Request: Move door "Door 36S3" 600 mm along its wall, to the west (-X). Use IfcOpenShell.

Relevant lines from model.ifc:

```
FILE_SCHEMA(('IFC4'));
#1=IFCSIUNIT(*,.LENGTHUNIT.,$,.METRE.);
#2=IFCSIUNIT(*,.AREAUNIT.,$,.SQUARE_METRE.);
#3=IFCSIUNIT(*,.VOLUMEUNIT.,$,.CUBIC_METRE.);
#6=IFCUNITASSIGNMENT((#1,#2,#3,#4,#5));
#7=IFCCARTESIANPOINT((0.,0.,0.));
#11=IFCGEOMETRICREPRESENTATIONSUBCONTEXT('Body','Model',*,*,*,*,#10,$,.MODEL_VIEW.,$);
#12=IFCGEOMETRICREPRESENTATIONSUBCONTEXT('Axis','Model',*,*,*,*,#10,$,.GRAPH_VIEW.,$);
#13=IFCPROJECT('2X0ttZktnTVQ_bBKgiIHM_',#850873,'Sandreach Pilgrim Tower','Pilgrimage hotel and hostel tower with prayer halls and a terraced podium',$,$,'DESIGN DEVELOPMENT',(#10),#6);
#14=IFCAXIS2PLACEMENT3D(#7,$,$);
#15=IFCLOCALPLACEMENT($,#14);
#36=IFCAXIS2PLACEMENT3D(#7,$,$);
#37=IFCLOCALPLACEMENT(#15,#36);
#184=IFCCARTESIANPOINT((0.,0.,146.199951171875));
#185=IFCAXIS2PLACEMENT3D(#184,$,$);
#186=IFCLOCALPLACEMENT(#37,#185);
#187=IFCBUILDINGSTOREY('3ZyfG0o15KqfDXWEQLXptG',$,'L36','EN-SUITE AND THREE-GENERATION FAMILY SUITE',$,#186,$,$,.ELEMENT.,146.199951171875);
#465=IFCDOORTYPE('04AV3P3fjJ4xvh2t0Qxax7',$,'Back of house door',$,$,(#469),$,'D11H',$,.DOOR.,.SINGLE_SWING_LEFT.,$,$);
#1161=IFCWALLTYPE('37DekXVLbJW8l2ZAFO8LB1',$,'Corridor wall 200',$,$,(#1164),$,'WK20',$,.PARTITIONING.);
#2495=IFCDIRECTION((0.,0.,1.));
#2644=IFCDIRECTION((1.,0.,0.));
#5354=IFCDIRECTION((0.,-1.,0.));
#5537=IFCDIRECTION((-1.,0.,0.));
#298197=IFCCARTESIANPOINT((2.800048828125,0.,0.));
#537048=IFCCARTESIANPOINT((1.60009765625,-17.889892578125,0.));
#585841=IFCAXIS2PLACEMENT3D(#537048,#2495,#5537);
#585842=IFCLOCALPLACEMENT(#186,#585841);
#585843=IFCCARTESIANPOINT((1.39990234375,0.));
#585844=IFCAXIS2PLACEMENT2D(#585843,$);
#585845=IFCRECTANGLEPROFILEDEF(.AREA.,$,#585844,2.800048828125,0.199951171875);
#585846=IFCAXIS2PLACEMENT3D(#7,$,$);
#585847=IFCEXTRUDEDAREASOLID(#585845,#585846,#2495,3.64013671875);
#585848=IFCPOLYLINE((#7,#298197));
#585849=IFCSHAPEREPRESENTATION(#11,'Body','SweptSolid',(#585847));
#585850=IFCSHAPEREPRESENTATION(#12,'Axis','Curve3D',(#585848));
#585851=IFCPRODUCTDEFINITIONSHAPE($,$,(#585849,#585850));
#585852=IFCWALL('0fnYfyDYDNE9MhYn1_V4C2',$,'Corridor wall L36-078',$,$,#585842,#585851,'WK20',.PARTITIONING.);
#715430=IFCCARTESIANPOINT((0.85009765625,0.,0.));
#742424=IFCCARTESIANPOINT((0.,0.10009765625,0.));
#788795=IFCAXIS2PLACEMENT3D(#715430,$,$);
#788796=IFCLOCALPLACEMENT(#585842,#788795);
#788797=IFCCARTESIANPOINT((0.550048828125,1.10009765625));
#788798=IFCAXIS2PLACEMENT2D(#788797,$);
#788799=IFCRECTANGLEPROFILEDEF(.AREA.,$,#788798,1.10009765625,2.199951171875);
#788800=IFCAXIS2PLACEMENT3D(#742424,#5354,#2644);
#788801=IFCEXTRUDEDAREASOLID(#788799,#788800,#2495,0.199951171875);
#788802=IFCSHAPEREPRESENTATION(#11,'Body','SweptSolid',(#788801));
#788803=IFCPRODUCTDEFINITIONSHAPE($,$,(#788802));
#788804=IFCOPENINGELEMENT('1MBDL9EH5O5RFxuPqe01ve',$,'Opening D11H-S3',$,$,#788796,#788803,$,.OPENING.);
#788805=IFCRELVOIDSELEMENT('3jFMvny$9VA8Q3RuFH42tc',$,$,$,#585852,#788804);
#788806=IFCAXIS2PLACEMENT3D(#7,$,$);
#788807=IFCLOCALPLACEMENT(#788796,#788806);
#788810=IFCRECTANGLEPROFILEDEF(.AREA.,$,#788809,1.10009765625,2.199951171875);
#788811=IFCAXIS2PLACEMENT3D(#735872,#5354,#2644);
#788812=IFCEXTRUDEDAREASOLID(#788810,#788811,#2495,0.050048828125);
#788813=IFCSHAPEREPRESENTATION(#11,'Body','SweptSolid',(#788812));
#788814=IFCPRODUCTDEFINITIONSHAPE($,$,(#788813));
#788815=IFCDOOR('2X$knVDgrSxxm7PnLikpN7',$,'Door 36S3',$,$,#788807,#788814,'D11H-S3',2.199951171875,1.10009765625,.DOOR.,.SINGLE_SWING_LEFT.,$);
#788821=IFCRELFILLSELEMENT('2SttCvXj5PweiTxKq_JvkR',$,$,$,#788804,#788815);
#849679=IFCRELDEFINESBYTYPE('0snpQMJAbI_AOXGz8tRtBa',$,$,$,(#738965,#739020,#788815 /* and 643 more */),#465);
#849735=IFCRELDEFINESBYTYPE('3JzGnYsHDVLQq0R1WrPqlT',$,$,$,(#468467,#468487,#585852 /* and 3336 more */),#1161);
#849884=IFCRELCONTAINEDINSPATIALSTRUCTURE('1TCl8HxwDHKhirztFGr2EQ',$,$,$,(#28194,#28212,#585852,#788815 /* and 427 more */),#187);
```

```python
import ifcopenshell
import ifcopenshell.api.geometry
import ifcopenshell.util.placement
import ifcopenshell.util.unit

model = ifcopenshell.open("model.ifc")
unit_scale = ifcopenshell.util.unit.calculate_unit_scale(model)

door = model.by_id(788815)
opening = door.FillsVoids[0].RelatingOpeningElement
wall = opening.VoidsElements[0].RelatingBuildingElement

wall_matrix = ifcopenshell.util.placement.get_local_placement(wall.ObjectPlacement)
shift = wall_matrix[:3, 0] * 0.6 / unit_scale
before = ifcopenshell.util.placement.get_local_placement(door.ObjectPlacement)[:3, 3].copy()

# The door is placed relative to its opening, so it follows when the opening moves.
matrix = ifcopenshell.util.placement.get_local_placement(opening.ObjectPlacement)
matrix[:3, 3] += shift
ifcopenshell.api.geometry.edit_object_placement(
    model, product=opening, matrix=matrix, is_si=False, should_transform_children=True
)

after = ifcopenshell.util.placement.get_local_placement(door.ObjectPlacement)[:3, 3]
print("door moved by", (after - before).round(3) + 0.0)

model.write("model-out.ifc")
```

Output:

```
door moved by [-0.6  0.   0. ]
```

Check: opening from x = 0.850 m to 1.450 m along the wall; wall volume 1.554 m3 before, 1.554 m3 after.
